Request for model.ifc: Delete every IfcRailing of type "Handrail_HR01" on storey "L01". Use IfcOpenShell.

First a look at what the model holds.

```python
import ifcopenshell
import ifcopenshell.util.element

model = ifcopenshell.open("model.ifc")
print(model.schema)
storey = next(s for s in model.by_type("IfcBuildingStorey") if s.Name == "L01")
railings = [e for e in ifcopenshell.util.element.get_decomposition(storey) if e.is_a("IfcRailing")]
seen = {}
for e in railings:
    element_type = ifcopenshell.util.element.get_type(e)
    name = element_type.Name if element_type not in (None, e) else None
    seen[name] = seen.get(name, 0) + 1
for name, count in sorted(seen.items(), key=str):
    print(count, "x", name)
```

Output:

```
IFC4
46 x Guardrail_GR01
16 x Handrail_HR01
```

```python
import ifcopenshell
import ifcopenshell.api.root
import ifcopenshell.util.element

model = ifcopenshell.open("model.ifc")

storey = next(s for s in model.by_type("IfcBuildingStorey") if s.Name == "L01")
railings = [e for e in ifcopenshell.util.element.get_decomposition(storey) if e.is_a("IfcRailing")]
targets = [e for e in railings if (t := ifcopenshell.util.element.get_type(e)) not in (None, e) and t.Name == "Handrail_HR01"]

for e in targets:
    ifcopenshell.api.root.remove_product(model, product=e)
print(len(targets), "removed")

model.write("model-out.ifc")
```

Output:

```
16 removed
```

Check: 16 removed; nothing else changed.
